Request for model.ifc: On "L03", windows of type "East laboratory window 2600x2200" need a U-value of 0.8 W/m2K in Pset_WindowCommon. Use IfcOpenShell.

First a look at what the model holds.

```python
import ifcopenshell
import ifcopenshell.util.element

model = ifcopenshell.open("model.ifc")
print(model.schema)
storey = next(s for s in model.by_type("IfcBuildingStorey") if s.Name == "L03")
windows = [e for e in ifcopenshell.util.element.get_decomposition(storey) if e.is_a("IfcWindow")]
seen = {}
for e in windows:
    element_type = ifcopenshell.util.element.get_type(e)
    key = (element_type.Name if element_type != e and element_type else None, ifcopenshell.util.element.get_pset(e, "Pset_WindowCommon", "ThermalTransmittance"))
    seen[key] = seen.get(key, 0) + 1
for (name, value), count in sorted(seen.items(), key=str):
    print(count, "x", name, "|", value)
```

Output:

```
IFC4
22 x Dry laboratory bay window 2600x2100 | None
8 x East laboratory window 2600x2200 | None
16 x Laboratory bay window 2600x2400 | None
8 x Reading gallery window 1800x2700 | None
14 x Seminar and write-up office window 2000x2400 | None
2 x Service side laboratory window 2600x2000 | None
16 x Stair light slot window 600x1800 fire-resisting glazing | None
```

```python
import ifcopenshell
import ifcopenshell.api.pset
import ifcopenshell.util.element

model = ifcopenshell.open("model.ifc")

storey = next(s for s in model.by_type("IfcBuildingStorey") if s.Name == "L03")
windows = [e for e in ifcopenshell.util.element.get_decomposition(storey) if e.is_a("IfcWindow")]

count = 0
for e in windows:
    element_type = ifcopenshell.util.element.get_type(e)
    if element_type in (None, e) or element_type.Name != "East laboratory window 2600x2200":
        continue
    # add_pset returns the element's existing set when there is one.
    pset = ifcopenshell.api.pset.add_pset(model, product=e, name="Pset_WindowCommon")
    ifcopenshell.api.pset.edit_pset(model, pset=pset, properties={"ThermalTransmittance": 0.8})
    count += 1

print(count, "windows updated")

model.write("model_v2.ifc")
```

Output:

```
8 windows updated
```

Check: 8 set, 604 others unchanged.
